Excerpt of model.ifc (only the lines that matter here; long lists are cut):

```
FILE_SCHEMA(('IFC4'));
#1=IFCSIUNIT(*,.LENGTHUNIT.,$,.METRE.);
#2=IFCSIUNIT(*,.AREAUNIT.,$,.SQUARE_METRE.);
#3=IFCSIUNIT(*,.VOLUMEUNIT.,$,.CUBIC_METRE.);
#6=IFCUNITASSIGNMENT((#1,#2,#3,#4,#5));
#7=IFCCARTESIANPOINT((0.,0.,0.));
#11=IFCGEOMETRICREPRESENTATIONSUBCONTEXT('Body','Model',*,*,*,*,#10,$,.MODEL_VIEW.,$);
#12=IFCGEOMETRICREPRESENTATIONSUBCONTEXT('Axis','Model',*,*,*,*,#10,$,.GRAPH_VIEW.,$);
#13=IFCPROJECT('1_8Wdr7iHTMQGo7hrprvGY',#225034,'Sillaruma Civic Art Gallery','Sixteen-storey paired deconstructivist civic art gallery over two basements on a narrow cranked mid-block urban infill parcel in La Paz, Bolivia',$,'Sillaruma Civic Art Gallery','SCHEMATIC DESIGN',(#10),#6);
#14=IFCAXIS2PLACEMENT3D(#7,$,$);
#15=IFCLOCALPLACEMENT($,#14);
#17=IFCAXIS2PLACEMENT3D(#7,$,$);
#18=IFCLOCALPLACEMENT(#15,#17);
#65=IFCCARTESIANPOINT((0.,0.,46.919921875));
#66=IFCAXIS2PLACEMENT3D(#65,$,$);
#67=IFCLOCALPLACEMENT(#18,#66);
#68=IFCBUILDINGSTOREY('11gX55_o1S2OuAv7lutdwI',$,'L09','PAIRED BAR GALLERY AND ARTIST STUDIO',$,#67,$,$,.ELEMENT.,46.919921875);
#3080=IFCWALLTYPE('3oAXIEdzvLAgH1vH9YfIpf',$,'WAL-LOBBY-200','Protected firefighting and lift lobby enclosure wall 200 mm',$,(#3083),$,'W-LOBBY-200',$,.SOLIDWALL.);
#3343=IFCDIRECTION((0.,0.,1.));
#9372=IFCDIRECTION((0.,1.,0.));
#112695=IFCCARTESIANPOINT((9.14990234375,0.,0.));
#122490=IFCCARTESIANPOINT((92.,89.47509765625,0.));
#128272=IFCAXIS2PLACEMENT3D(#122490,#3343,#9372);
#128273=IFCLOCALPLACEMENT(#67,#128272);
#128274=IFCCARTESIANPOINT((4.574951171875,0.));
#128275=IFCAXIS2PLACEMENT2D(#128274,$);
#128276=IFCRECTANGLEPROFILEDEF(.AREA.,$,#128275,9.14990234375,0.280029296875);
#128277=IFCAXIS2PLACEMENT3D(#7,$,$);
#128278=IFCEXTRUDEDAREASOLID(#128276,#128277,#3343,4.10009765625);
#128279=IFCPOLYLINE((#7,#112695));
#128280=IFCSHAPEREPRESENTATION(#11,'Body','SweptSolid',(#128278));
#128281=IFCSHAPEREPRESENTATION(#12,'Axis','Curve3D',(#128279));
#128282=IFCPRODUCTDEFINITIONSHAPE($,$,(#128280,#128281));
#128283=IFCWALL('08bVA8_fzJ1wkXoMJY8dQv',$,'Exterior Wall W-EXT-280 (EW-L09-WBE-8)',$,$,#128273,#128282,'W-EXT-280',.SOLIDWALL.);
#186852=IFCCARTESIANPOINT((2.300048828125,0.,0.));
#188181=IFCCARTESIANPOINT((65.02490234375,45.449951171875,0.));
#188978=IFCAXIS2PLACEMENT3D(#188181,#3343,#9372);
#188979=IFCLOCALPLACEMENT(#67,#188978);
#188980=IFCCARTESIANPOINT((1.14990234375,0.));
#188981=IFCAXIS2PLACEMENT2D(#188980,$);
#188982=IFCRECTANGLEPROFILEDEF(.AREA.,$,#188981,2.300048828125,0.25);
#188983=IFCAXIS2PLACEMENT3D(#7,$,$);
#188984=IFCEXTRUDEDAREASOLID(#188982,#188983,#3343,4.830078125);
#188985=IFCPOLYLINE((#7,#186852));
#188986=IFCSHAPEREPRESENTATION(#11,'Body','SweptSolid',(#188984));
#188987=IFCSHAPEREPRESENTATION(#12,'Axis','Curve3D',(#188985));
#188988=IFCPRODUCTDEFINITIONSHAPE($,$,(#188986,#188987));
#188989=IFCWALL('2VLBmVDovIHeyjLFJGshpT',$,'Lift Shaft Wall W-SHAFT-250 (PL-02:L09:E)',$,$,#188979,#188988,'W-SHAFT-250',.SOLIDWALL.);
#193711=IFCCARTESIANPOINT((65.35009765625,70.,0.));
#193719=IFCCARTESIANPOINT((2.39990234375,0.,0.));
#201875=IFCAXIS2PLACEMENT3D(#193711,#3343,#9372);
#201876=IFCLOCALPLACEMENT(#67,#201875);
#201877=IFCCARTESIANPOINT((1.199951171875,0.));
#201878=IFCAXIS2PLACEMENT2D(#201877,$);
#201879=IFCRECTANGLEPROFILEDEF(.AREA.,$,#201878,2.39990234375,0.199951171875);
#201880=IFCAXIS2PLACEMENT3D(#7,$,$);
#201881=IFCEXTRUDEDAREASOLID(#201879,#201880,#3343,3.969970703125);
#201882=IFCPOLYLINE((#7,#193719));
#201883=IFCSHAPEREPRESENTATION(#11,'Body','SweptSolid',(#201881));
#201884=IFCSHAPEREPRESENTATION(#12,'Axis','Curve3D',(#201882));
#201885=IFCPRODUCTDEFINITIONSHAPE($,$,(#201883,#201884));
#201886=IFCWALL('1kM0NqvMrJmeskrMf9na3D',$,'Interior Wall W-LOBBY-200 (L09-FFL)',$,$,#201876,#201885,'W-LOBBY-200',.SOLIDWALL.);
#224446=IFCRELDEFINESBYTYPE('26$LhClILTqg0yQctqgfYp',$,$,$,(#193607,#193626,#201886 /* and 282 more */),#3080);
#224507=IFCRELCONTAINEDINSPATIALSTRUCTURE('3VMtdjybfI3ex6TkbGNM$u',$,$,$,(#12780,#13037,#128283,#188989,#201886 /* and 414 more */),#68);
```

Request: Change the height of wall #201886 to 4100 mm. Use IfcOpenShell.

```python
import ifcopenshell
import ifcopenshell.geom
import ifcopenshell.util.representation
import ifcopenshell.util.shape

model = ifcopenshell.open("model.ifc")
settings = ifcopenshell.geom.settings()


def volume(element):
    """Net volume in cubic metres, openings subtracted."""
    shape = ifcopenshell.geom.create_shape(settings, element)
    return ifcopenshell.util.shape.get_volume(shape.geometry)


wall = model.by_id(201886)
before = volume(wall)

body = ifcopenshell.util.representation.get_representation(wall, "Model", "Body")
solid = body.Items[0]
old_height = solid.Depth
solid.Depth = 4.1
after = volume(wall)

print(f"height {old_height:g} -> {solid.Depth:g}, volume {before:.3f} -> {after:.3f} m3")

model.write("model_rev.ifc")
```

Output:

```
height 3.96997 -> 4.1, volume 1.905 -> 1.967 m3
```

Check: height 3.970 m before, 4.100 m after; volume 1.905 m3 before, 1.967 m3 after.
